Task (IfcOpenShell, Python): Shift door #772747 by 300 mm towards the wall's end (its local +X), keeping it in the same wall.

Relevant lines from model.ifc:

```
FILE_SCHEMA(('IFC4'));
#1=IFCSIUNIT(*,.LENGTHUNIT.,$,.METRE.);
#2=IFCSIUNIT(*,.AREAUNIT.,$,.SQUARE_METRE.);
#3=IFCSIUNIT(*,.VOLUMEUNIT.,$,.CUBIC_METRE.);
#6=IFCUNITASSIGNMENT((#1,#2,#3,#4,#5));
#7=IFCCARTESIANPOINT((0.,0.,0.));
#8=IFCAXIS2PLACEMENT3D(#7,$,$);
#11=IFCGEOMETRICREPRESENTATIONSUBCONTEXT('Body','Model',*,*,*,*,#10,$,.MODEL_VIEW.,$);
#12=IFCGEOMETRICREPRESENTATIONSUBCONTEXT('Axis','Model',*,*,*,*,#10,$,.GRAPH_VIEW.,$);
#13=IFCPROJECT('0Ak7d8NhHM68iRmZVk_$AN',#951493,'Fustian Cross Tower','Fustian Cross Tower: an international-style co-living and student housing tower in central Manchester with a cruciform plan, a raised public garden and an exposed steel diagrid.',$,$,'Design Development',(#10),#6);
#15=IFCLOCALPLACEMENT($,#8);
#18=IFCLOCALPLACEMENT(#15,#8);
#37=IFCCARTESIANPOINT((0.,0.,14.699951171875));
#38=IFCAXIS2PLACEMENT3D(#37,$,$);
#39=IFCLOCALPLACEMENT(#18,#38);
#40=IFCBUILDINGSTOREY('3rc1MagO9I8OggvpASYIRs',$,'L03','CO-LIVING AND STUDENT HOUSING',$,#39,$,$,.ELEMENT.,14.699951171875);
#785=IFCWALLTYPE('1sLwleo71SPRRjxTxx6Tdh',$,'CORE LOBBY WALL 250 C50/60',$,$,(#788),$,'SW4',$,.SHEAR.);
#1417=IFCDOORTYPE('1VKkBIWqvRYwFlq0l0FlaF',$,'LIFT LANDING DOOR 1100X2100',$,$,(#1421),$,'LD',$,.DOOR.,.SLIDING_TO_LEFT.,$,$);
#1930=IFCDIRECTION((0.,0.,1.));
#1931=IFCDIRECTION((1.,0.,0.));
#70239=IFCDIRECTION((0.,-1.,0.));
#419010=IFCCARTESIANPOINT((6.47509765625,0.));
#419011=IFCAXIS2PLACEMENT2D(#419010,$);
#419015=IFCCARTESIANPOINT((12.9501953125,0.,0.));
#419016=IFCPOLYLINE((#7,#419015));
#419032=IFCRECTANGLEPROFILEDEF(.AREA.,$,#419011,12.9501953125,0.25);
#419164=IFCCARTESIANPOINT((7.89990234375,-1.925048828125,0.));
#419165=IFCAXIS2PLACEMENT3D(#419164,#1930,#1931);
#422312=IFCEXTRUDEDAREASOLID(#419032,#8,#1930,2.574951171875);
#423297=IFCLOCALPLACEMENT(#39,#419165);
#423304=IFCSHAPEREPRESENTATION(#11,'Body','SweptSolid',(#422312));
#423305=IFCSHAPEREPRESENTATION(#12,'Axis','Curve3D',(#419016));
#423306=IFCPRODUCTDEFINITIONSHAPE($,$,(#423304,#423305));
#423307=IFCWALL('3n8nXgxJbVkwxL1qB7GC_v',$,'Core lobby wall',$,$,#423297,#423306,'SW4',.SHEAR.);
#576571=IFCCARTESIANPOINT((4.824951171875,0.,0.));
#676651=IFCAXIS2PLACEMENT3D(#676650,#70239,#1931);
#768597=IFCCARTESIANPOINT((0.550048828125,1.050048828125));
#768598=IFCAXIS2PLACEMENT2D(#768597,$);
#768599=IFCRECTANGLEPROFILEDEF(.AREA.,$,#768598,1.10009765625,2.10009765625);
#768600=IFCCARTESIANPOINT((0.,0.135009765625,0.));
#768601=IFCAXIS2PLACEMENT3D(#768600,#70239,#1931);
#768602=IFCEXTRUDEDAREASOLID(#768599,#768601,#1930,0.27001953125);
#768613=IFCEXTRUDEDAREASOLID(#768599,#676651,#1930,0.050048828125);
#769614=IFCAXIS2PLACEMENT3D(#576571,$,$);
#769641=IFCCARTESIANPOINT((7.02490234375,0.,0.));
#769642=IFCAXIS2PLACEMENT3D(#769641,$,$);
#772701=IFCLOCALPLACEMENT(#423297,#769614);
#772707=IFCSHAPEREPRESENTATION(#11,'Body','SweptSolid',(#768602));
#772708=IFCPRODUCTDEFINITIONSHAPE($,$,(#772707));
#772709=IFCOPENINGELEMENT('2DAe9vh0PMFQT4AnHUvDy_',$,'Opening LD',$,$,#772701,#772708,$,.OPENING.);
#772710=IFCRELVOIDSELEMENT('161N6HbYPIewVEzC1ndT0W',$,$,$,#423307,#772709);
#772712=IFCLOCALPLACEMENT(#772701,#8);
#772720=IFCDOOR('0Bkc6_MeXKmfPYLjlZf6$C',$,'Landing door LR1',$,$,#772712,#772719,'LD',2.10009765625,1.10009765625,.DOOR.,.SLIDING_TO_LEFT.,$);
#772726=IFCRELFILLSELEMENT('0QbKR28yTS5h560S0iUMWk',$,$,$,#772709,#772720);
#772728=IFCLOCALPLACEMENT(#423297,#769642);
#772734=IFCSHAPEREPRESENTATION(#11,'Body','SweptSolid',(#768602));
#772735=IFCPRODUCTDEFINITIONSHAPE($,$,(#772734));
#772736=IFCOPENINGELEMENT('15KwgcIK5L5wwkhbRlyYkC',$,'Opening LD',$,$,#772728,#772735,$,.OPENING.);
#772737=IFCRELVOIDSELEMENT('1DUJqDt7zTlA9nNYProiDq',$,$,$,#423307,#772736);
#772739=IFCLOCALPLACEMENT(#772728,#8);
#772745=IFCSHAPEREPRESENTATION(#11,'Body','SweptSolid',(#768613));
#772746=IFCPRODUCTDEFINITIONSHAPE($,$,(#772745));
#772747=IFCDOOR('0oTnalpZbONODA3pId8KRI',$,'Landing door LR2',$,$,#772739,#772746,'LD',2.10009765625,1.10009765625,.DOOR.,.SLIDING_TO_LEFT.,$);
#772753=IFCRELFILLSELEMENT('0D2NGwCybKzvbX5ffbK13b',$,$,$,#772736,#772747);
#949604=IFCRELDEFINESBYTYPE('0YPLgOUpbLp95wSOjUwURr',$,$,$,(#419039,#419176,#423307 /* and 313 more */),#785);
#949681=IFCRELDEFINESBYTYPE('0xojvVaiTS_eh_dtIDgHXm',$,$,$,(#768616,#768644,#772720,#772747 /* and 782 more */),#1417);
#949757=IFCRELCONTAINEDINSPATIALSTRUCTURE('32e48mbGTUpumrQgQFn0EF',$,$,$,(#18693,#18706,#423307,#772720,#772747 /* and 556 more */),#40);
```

```python
import ifcopenshell
import ifcopenshell.api.geometry
import ifcopenshell.util.placement
import ifcopenshell.util.unit

model = ifcopenshell.open("model.ifc")
unit_scale = ifcopenshell.util.unit.calculate_unit_scale(model)

door = model.by_guid("0oTnalpZbONODA3pId8KRI")
opening = door.FillsVoids[0].RelatingOpeningElement
wall = opening.VoidsElements[0].RelatingBuildingElement

wall_matrix = ifcopenshell.util.placement.get_local_placement(wall.ObjectPlacement)
shift = wall_matrix[:3, 0] * 0.3 / unit_scale
before = ifcopenshell.util.placement.get_local_placement(door.ObjectPlacement)[:3, 3].copy()

# The door is placed relative to its opening, so it follows when the opening moves.
matrix = ifcopenshell.util.placement.get_local_placement(opening.ObjectPlacement)
matrix[:3, 3] += shift
ifcopenshell.api.geometry.edit_object_placement(
    model, product=opening, matrix=matrix, is_si=False, should_transform_children=True
)

after = ifcopenshell.util.placement.get_local_placement(door.ObjectPlacement)[:3, 3]
print("door moved by", (after - before).round(3) + 0.0)

model.write("model_v2.ifc")
```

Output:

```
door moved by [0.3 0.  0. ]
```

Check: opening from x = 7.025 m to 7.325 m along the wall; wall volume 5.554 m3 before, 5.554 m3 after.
